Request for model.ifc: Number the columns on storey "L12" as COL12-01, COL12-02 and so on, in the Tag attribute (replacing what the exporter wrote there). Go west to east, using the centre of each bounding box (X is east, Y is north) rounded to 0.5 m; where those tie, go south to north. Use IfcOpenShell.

First a look at what the model holds.

```python
import ifcopenshell
import ifcopenshell.util.element
import ifcopenshell.util.placement

model = ifcopenshell.open("model.ifc")
print(model.schema)
storey = next(s for s in model.by_type("IfcBuildingStorey") if s.Name == "L12")
columns = [e for e in ifcopenshell.util.element.get_decomposition(storey) if e.is_a("IfcColumn")]
for e in sorted(columns, key=lambda e: e.id()):
    origin = ifcopenshell.util.placement.get_local_placement(e.ObjectPlacement)[:3, 3]
    print(e.id(), e.Tag, e.Name, origin.round(2) + 0.0, sep=" | ")
```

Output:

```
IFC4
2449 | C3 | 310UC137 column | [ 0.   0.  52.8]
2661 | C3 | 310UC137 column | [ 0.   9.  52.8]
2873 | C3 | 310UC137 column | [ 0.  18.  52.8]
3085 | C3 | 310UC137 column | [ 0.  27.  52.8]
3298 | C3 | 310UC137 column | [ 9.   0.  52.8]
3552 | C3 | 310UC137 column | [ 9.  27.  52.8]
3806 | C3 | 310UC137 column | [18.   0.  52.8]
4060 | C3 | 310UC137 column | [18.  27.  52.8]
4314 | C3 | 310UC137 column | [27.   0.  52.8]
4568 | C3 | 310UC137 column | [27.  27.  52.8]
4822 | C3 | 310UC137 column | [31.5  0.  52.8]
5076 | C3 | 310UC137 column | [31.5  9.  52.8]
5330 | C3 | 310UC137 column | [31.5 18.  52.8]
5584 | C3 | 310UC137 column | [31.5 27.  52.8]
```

```python
import ifcopenshell
import ifcopenshell.geom
import ifcopenshell.util.element
import ifcopenshell.util.shape

model = ifcopenshell.open("model.ifc")
settings = ifcopenshell.geom.settings()
settings.set("use-world-coords", True)


def centre(element):
    shape = ifcopenshell.geom.create_shape(settings, element)
    return ifcopenshell.util.shape.get_bbox_centroid(shape.geometry)


storey = next(s for s in model.by_type("IfcBuildingStorey") if s.Name == "L12")
columns = [e for e in ifcopenshell.util.element.get_decomposition(storey) if e.is_a("IfcColumn")]

# Insertion points can sit at a corner or the storey origin, so sort by the geometry (in metres).
centres = {e: centre(e) for e in columns}
columns.sort(key=lambda e: (round(centres[e][0] / 0.5), centres[e][1]))

for i, e in enumerate(columns, start=1):
    number = f"COL12-{i:02d}"
    e.Tag = number
    print(e.id(), number)

model.write("model_v2.ifc")
```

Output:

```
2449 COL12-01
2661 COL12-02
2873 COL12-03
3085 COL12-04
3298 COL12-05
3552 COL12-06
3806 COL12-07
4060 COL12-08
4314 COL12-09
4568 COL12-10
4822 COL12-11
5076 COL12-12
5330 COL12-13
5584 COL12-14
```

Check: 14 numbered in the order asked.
